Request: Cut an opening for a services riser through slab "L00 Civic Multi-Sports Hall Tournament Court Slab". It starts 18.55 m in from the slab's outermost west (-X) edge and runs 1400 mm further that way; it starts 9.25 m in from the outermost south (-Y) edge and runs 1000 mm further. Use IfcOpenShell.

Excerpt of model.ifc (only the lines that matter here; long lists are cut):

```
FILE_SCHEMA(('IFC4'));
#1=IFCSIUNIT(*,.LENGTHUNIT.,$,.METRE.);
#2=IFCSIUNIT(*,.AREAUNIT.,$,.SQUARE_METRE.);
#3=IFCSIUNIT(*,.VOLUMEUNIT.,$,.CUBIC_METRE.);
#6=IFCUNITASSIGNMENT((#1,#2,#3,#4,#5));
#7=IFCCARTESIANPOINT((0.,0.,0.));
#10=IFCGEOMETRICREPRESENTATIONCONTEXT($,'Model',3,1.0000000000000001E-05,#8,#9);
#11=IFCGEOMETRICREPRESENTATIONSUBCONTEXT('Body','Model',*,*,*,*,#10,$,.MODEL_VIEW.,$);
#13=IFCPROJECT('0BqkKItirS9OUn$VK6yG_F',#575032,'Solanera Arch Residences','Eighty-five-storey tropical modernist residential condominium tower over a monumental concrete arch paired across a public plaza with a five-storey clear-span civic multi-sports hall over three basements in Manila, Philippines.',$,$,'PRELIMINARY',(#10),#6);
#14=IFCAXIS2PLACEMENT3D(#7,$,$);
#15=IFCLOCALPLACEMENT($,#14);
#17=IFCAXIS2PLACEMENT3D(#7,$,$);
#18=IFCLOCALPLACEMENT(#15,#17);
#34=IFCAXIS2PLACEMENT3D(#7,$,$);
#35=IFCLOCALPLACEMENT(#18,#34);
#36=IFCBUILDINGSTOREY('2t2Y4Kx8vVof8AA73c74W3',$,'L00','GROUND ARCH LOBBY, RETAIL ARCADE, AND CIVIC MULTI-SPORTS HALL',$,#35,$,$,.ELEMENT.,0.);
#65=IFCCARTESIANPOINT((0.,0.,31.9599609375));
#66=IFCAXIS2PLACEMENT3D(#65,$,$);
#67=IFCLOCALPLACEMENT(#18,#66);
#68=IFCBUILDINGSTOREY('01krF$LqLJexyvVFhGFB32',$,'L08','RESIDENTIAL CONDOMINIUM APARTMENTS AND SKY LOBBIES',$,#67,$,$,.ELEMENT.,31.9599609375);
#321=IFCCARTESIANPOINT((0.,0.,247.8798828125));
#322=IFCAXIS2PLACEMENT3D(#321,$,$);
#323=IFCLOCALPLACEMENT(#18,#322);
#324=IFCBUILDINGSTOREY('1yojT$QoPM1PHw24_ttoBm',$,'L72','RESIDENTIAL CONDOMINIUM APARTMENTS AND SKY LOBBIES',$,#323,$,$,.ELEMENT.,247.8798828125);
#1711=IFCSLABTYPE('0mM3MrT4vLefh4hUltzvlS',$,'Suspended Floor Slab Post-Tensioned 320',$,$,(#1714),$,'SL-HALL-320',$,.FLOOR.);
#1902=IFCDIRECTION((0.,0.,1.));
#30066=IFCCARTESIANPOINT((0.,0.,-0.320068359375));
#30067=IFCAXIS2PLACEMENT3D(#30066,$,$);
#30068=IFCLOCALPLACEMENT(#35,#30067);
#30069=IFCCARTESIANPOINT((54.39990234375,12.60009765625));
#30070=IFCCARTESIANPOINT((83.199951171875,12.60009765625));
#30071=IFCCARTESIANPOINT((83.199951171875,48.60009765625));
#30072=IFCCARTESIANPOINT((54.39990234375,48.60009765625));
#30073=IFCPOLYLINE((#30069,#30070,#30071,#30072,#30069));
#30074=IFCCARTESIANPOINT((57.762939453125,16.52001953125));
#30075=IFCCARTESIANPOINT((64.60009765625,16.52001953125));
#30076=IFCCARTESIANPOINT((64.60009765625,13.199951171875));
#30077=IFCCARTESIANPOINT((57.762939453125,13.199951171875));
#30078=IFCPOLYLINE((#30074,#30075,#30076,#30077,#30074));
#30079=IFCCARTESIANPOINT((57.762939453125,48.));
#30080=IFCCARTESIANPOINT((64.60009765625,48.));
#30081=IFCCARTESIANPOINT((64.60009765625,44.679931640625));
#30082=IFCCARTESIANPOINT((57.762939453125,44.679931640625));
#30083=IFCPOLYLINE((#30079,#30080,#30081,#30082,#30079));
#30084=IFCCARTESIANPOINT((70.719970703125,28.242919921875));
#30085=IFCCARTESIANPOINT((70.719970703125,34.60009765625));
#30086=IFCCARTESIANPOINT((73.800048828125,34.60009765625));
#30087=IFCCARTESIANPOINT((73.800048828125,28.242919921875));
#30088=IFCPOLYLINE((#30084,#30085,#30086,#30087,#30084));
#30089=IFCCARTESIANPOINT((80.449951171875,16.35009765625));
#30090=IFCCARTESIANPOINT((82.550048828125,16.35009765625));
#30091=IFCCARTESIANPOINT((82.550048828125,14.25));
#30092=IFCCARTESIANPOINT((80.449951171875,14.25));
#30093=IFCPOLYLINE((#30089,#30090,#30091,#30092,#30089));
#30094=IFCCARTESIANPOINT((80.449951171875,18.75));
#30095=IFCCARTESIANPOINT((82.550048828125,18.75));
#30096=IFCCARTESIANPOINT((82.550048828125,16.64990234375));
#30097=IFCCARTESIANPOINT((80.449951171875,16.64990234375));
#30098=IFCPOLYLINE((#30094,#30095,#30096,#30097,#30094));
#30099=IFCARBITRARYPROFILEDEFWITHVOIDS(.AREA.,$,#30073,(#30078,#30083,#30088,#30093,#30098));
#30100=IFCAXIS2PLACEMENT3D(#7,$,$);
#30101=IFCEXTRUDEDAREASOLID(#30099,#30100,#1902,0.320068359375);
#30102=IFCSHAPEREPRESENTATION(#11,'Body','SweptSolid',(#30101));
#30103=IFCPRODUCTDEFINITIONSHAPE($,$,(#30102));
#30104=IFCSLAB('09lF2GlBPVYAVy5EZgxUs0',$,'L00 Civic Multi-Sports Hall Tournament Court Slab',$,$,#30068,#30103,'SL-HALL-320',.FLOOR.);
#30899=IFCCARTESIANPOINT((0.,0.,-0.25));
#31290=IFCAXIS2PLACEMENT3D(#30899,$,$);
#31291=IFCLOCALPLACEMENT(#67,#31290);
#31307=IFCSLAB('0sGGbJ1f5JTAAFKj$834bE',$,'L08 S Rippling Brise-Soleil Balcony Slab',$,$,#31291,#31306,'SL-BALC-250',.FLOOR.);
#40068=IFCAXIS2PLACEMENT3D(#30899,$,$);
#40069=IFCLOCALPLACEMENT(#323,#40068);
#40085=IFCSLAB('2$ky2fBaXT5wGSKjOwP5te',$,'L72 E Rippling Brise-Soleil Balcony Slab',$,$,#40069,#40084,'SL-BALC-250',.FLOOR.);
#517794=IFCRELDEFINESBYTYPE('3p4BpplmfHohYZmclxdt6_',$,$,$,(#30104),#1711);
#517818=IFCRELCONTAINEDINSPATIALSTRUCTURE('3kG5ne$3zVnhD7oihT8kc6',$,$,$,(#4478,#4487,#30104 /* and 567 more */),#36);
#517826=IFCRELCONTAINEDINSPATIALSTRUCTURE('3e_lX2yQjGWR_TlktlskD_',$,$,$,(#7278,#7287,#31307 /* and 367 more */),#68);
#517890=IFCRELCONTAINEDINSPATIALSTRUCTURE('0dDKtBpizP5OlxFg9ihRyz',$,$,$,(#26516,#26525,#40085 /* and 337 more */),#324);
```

```python
import numpy as np
import ifcopenshell
import ifcopenshell.api.feature
import ifcopenshell.api.geometry
import ifcopenshell.api.root
import ifcopenshell.geom
import ifcopenshell.util.placement
import ifcopenshell.util.representation
import ifcopenshell.util.shape
import ifcopenshell.util.unit

model = ifcopenshell.open("model.ifc")
unit_scale = ifcopenshell.util.unit.calculate_unit_scale(model)
settings = ifcopenshell.geom.settings()


def volume(element):
    """Net volume in cubic metres, openings subtracted."""
    shape = ifcopenshell.geom.create_shape(settings, element)
    return ifcopenshell.util.shape.get_volume(shape.geometry)


slab = model.by_id(30104)
before = volume(slab)

# Extent in the slab's own axes, in metres. The edges named are its -X and -Y sides.
slab_shape = ifcopenshell.geom.create_shape(settings, slab)
vertices = ifcopenshell.util.shape.get_vertices(slab_shape.geometry)
x_min, y_min, bottom = vertices.min(axis=0)
top = vertices[:, 2].max()

opening = ifcopenshell.api.root.create_entity(model, ifc_class="IfcOpeningElement", name="Services riser opening", predefined_type="OPENING")
context = ifcopenshell.util.representation.get_context(model, "Model", "Body", "MODEL_VIEW")
width, depth = 1.4, 1
outline = [(0.0, 0.0), (width, 0.0), (width, depth), (0.0, depth), (0.0, 0.0)]
# Overshoot both faces by 50 mm so the cut is clean.
shape = ifcopenshell.api.geometry.add_slab_representation(
    model, context=context, depth=top - bottom + 0.1, polyline=outline
)
ifcopenshell.api.geometry.assign_representation(model, product=opening, representation=shape)

matrix = ifcopenshell.util.placement.get_local_placement(slab.ObjectPlacement)
matrix[:, 3] = matrix @ np.append(np.array([x_min + 18.55, y_min + 9.25, bottom - 0.05]) / unit_scale, 1.0)
ifcopenshell.api.geometry.edit_object_placement(model, product=opening, matrix=matrix, is_si=False)
ifcopenshell.api.feature.add_feature(model, feature=opening, element=slab)

after = volume(slab)

print(f"slab volume {before:.3f} -> {after:.3f} m3")

model.write("model_edited.ifc")
```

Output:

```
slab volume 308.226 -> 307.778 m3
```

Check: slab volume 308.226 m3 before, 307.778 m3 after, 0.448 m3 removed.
